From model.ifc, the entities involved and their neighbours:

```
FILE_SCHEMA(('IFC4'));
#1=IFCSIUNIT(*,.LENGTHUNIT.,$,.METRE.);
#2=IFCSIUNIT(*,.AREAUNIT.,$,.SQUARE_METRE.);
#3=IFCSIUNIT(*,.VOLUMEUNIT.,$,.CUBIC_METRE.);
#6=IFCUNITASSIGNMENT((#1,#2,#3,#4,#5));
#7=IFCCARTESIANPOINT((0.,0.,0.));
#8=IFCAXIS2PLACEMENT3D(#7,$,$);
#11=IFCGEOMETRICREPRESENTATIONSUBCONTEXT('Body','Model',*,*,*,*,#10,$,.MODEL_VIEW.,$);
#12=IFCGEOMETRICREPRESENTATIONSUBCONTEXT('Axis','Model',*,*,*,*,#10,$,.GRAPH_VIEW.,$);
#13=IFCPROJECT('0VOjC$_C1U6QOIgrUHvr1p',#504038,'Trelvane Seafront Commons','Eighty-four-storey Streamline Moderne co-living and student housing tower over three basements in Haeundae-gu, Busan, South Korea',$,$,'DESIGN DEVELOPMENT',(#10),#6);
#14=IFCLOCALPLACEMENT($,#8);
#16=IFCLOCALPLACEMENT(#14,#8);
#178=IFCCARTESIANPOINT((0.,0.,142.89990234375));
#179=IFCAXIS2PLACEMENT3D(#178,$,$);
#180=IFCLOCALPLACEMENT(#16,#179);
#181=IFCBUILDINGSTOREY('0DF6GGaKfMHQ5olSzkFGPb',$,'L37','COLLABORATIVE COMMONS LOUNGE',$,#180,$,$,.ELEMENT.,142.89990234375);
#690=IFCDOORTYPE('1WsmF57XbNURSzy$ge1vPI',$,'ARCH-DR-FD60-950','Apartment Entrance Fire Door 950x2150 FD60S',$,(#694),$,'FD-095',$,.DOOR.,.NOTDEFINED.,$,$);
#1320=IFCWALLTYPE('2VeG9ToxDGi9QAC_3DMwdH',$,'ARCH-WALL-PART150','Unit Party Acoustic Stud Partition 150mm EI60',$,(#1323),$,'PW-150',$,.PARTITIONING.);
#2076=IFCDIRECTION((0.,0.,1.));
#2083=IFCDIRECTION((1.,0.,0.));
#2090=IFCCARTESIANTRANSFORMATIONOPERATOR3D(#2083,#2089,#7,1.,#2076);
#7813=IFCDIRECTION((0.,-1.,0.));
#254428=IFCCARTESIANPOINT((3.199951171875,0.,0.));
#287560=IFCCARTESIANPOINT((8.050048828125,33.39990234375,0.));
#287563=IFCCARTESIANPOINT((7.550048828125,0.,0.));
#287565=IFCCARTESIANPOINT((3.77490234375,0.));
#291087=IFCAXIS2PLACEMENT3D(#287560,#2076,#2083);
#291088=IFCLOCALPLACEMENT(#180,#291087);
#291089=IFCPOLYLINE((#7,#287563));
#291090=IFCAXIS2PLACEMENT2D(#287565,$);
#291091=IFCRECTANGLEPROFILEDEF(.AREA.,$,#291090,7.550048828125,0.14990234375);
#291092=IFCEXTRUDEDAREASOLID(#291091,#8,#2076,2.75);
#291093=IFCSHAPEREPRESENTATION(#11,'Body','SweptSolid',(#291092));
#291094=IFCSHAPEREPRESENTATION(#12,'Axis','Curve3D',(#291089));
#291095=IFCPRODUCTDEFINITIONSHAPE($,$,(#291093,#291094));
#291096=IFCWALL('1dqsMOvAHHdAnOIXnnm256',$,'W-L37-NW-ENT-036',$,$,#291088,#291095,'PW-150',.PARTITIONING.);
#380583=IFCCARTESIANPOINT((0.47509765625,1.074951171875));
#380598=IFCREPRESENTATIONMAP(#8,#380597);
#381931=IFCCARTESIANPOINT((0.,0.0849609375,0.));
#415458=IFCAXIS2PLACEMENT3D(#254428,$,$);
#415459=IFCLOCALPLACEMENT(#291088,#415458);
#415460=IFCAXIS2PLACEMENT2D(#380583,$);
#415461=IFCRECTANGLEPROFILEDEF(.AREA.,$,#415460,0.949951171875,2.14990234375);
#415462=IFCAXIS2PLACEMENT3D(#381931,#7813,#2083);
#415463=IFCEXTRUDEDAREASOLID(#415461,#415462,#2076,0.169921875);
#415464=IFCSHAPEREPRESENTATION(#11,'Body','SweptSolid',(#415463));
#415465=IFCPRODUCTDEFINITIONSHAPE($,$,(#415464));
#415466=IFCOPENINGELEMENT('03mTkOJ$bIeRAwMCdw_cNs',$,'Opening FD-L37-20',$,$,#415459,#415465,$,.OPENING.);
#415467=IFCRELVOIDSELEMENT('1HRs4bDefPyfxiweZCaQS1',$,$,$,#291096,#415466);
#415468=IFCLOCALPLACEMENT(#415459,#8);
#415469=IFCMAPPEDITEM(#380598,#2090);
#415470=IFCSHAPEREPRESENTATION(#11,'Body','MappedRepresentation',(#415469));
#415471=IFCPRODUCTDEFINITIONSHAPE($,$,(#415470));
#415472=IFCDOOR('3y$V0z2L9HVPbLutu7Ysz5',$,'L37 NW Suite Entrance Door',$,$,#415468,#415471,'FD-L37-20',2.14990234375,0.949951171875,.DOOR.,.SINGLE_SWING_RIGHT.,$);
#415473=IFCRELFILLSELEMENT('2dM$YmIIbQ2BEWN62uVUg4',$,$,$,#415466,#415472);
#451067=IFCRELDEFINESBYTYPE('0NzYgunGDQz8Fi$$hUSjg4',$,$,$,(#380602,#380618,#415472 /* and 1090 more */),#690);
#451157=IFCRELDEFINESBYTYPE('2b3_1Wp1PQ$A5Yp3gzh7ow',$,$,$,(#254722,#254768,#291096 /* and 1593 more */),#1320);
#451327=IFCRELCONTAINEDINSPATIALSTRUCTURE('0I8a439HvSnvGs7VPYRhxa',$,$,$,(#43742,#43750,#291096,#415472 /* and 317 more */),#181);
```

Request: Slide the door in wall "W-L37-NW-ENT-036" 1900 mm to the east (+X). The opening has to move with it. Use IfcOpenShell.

```python
import ifcopenshell
import ifcopenshell.api.geometry
import ifcopenshell.util.placement
import ifcopenshell.util.unit

model = ifcopenshell.open("model.ifc")
unit_scale = ifcopenshell.util.unit.calculate_unit_scale(model)

door = model.by_guid("3y$V0z2L9HVPbLutu7Ysz5")
opening = door.FillsVoids[0].RelatingOpeningElement
wall = opening.VoidsElements[0].RelatingBuildingElement

wall_matrix = ifcopenshell.util.placement.get_local_placement(wall.ObjectPlacement)
shift = wall_matrix[:3, 0] * 1.9 / unit_scale
before = ifcopenshell.util.placement.get_local_placement(door.ObjectPlacement)[:3, 3].copy()

# The door is placed relative to its opening, so it follows when the opening moves.
matrix = ifcopenshell.util.placement.get_local_placement(opening.ObjectPlacement)
matrix[:3, 3] += shift
ifcopenshell.api.geometry.edit_object_placement(
    model, product=opening, matrix=matrix, is_si=False, should_transform_children=True
)

after = ifcopenshell.util.placement.get_local_placement(door.ObjectPlacement)[:3, 3]
print("door moved by", (after - before).round(3) + 0.0)

model.write("model-out.ifc")
```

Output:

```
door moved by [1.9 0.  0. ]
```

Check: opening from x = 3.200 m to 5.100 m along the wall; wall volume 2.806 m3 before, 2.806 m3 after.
